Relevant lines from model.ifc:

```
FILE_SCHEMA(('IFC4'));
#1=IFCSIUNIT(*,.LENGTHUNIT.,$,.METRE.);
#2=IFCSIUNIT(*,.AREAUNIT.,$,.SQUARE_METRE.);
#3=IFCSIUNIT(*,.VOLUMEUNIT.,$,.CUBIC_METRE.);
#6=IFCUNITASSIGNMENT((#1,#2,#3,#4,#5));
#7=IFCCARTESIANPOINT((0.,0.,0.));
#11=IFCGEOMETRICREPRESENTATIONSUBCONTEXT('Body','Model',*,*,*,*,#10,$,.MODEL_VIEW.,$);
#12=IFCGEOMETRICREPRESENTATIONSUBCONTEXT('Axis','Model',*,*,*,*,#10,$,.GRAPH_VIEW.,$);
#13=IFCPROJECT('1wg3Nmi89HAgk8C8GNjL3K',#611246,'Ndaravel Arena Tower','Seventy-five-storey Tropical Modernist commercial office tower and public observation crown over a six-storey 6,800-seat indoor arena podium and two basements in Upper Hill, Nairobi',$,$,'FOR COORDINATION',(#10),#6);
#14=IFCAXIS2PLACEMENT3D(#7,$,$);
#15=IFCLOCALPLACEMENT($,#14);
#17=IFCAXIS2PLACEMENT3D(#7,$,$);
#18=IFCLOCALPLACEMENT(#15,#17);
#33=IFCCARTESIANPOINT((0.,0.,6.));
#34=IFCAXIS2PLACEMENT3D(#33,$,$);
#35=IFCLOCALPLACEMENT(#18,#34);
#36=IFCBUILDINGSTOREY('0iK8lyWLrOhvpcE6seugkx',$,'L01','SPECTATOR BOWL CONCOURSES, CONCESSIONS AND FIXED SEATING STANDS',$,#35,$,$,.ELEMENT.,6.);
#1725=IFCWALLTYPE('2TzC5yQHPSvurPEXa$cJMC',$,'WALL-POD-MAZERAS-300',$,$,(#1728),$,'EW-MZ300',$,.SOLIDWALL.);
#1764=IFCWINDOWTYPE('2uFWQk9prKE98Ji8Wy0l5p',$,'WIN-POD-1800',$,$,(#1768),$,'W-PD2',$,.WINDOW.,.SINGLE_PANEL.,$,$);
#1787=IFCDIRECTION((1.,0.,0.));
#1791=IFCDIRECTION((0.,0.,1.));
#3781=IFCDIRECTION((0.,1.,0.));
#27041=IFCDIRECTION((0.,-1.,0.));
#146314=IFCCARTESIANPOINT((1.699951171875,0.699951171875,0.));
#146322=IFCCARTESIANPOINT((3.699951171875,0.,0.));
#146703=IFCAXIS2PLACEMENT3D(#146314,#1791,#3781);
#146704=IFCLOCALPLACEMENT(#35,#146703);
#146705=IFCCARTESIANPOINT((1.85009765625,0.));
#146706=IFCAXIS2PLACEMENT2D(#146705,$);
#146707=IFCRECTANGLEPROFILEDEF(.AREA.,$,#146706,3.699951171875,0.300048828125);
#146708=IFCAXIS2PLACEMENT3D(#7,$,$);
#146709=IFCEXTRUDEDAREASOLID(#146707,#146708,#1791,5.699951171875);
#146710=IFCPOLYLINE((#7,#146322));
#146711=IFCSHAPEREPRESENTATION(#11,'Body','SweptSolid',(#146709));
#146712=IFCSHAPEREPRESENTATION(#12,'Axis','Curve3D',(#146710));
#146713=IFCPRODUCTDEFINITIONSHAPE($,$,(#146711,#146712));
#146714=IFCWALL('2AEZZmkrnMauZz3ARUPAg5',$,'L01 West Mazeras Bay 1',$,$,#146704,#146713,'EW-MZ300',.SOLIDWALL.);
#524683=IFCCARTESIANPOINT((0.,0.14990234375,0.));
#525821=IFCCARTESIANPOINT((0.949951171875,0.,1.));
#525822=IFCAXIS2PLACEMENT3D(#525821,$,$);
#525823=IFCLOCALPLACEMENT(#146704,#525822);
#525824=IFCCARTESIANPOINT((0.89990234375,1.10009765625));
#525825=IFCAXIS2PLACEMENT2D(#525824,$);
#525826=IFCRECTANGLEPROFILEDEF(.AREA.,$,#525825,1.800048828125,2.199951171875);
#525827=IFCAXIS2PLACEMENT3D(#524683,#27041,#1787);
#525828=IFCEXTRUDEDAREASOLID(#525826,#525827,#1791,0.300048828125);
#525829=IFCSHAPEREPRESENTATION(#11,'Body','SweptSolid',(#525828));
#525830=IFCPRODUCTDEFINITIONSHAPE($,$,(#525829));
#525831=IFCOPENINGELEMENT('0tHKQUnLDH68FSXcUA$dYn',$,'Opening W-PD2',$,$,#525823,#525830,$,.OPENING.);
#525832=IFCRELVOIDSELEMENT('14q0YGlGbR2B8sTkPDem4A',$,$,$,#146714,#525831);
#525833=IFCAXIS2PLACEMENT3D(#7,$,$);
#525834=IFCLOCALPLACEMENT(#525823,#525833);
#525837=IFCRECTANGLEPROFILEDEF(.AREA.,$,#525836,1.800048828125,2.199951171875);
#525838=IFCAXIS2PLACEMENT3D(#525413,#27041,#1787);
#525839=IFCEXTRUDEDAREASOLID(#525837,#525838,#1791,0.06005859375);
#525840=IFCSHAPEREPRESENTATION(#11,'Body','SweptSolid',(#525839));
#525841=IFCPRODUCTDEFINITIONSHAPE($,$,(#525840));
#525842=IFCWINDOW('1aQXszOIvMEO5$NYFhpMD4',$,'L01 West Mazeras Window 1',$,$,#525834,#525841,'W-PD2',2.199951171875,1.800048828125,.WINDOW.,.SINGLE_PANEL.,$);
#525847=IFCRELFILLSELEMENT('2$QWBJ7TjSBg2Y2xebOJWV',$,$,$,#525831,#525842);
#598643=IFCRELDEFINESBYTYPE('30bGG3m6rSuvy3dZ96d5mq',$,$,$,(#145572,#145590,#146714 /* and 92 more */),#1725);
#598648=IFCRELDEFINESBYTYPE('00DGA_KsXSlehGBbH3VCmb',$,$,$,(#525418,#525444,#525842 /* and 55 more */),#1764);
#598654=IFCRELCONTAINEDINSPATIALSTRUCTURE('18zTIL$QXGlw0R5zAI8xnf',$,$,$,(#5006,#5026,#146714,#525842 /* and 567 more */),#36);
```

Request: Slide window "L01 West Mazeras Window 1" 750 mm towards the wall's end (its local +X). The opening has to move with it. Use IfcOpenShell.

```python
import ifcopenshell
import ifcopenshell.api.geometry
import ifcopenshell.util.placement

model = ifcopenshell.open("model.ifc")

window = model.by_guid("1aQXszOIvMEO5$NYFhpMD4")
opening = window.FillsVoids[0].RelatingOpeningElement
wall = opening.VoidsElements[0].RelatingBuildingElement

wall_matrix = ifcopenshell.util.placement.get_local_placement(wall.ObjectPlacement)
shift = wall_matrix[:3, 0] * 0.75
before = ifcopenshell.util.placement.get_local_placement(window.ObjectPlacement)[:3, 3].copy()

# The window is placed relative to its opening, so it follows when the opening moves.
matrix = ifcopenshell.util.placement.get_local_placement(opening.ObjectPlacement)
matrix[:3, 3] += shift
ifcopenshell.api.geometry.edit_object_placement(
    model, product=opening, matrix=matrix, is_si=False, should_transform_children=True
)

after = ifcopenshell.util.placement.get_local_placement(window.ObjectPlacement)[:3, 3]
print("window moved by", (after - before).round(3) + 0.0)

model.write("model_updated.ifc")
```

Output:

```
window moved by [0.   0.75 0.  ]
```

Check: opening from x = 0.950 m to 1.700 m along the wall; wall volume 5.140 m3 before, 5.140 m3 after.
